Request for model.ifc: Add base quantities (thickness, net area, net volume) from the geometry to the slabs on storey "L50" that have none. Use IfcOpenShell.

First a look at what the model holds.

```python
import ifcopenshell
import ifcopenshell.util.element
import ifcopenshell.util.unit

model = ifcopenshell.open("model.ifc")
print(model.schema)
for unit_type in ("LENGTHUNIT", "AREAUNIT", "VOLUMEUNIT"):
    print(unit_type, ifcopenshell.util.unit.calculate_unit_scale(model, unit_type))
storey = next(s for s in model.by_type("IfcBuildingStorey") if s.Name == "L50")
slabs = [e for e in ifcopenshell.util.element.get_decomposition(storey) if e.is_a("IfcSlab")]
for e in sorted(slabs, key=lambda e: e.id()):
    print(e.id(), e.is_a(), e.Name, list(ifcopenshell.util.element.get_psets(e, qtos_only=True)), sep=" | ")
```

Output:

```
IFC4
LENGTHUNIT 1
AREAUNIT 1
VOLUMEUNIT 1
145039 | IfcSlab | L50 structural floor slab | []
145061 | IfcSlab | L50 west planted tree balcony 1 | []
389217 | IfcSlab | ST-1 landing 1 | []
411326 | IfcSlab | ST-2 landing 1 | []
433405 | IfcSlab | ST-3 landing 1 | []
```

```python
import ifcopenshell
import ifcopenshell.api.pset
import ifcopenshell.geom
import ifcopenshell.util.element
import ifcopenshell.util.shape
import ifcopenshell.util.unit

model = ifcopenshell.open("model.ifc")
unit_scale = ifcopenshell.util.unit.calculate_unit_scale(model)
area_scale = ifcopenshell.util.unit.calculate_unit_scale(model, "AREAUNIT")
volume_scale = ifcopenshell.util.unit.calculate_unit_scale(model, "VOLUMEUNIT")
settings = ifcopenshell.geom.settings()

storey = next(s for s in model.by_type("IfcBuildingStorey") if s.Name == "L50")
slabs = [e for e in ifcopenshell.util.element.get_decomposition(storey) if e.is_a("IfcSlab")]

for e in sorted(slabs, key=lambda e: e.id()):
    if ifcopenshell.util.element.get_psets(e, qtos_only=True, should_inherit=False):
        continue
    # Geometry comes back in metres, in the element's own axes.
    shape = ifcopenshell.geom.create_shape(settings, e)
    values = {
        "Width": ifcopenshell.util.shape.get_z(shape.geometry) / unit_scale,
        "NetArea": ifcopenshell.util.shape.get_footprint_area(shape.geometry) / area_scale,
        "NetVolume": ifcopenshell.util.shape.get_volume(shape.geometry) / volume_scale,
    }
    qto = ifcopenshell.api.pset.add_qto(model, product=e, name="Qto_SlabBaseQuantities")
    ifcopenshell.api.pset.edit_qto(model, qto=qto, properties=values)
    print(e.id(), {k: round(v, 3) for k, v in values.items()})

model.write("model_rev.ifc")
```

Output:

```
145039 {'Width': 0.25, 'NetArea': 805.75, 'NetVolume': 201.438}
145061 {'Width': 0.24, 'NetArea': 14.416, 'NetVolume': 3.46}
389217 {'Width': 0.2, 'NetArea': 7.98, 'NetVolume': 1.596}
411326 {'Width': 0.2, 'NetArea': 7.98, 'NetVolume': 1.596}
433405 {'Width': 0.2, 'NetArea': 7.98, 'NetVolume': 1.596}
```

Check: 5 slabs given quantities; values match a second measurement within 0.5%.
